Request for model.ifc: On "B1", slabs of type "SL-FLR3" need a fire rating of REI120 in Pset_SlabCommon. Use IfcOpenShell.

First a look at what the model holds.

```python
import ifcopenshell
import ifcopenshell.util.element

model = ifcopenshell.open("model.ifc")
print(model.schema)
storey = next(s for s in model.by_type("IfcBuildingStorey") if s.Name == "B1")
slabs = [e for e in ifcopenshell.util.element.get_decomposition(storey) if e.is_a("IfcSlab")]
seen = {}
for e in slabs:
    element_type = ifcopenshell.util.element.get_type(e)
    key = (element_type.Name if element_type != e and element_type else None, ifcopenshell.util.element.get_pset(e, "Pset_SlabCommon", "FireRating"))
    seen[key] = seen.get(key, 0) + 1
for (name, value), count in sorted(seen.items(), key=str):
    print(count, "x", name, "|", value)
```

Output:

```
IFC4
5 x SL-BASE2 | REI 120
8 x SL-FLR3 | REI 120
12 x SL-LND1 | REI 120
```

```python
import ifcopenshell
import ifcopenshell.api.pset
import ifcopenshell.util.element

model = ifcopenshell.open("model.ifc")

storey = next(s for s in model.by_type("IfcBuildingStorey") if s.Name == "B1")
slabs = [e for e in ifcopenshell.util.element.get_decomposition(storey) if e.is_a("IfcSlab")]

count = 0
for e in slabs:
    element_type = ifcopenshell.util.element.get_type(e)
    if element_type in (None, e) or element_type.Name != "SL-FLR3":
        continue
    # add_pset returns the element's existing set when there is one.
    pset = ifcopenshell.api.pset.add_pset(model, product=e, name="Pset_SlabCommon")
    ifcopenshell.api.pset.edit_pset(model, pset=pset, properties={"FireRating": "REI120"})
    count += 1

print(count, "slabs updated")

model.write("model_edited.ifc")
```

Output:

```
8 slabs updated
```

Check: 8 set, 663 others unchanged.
